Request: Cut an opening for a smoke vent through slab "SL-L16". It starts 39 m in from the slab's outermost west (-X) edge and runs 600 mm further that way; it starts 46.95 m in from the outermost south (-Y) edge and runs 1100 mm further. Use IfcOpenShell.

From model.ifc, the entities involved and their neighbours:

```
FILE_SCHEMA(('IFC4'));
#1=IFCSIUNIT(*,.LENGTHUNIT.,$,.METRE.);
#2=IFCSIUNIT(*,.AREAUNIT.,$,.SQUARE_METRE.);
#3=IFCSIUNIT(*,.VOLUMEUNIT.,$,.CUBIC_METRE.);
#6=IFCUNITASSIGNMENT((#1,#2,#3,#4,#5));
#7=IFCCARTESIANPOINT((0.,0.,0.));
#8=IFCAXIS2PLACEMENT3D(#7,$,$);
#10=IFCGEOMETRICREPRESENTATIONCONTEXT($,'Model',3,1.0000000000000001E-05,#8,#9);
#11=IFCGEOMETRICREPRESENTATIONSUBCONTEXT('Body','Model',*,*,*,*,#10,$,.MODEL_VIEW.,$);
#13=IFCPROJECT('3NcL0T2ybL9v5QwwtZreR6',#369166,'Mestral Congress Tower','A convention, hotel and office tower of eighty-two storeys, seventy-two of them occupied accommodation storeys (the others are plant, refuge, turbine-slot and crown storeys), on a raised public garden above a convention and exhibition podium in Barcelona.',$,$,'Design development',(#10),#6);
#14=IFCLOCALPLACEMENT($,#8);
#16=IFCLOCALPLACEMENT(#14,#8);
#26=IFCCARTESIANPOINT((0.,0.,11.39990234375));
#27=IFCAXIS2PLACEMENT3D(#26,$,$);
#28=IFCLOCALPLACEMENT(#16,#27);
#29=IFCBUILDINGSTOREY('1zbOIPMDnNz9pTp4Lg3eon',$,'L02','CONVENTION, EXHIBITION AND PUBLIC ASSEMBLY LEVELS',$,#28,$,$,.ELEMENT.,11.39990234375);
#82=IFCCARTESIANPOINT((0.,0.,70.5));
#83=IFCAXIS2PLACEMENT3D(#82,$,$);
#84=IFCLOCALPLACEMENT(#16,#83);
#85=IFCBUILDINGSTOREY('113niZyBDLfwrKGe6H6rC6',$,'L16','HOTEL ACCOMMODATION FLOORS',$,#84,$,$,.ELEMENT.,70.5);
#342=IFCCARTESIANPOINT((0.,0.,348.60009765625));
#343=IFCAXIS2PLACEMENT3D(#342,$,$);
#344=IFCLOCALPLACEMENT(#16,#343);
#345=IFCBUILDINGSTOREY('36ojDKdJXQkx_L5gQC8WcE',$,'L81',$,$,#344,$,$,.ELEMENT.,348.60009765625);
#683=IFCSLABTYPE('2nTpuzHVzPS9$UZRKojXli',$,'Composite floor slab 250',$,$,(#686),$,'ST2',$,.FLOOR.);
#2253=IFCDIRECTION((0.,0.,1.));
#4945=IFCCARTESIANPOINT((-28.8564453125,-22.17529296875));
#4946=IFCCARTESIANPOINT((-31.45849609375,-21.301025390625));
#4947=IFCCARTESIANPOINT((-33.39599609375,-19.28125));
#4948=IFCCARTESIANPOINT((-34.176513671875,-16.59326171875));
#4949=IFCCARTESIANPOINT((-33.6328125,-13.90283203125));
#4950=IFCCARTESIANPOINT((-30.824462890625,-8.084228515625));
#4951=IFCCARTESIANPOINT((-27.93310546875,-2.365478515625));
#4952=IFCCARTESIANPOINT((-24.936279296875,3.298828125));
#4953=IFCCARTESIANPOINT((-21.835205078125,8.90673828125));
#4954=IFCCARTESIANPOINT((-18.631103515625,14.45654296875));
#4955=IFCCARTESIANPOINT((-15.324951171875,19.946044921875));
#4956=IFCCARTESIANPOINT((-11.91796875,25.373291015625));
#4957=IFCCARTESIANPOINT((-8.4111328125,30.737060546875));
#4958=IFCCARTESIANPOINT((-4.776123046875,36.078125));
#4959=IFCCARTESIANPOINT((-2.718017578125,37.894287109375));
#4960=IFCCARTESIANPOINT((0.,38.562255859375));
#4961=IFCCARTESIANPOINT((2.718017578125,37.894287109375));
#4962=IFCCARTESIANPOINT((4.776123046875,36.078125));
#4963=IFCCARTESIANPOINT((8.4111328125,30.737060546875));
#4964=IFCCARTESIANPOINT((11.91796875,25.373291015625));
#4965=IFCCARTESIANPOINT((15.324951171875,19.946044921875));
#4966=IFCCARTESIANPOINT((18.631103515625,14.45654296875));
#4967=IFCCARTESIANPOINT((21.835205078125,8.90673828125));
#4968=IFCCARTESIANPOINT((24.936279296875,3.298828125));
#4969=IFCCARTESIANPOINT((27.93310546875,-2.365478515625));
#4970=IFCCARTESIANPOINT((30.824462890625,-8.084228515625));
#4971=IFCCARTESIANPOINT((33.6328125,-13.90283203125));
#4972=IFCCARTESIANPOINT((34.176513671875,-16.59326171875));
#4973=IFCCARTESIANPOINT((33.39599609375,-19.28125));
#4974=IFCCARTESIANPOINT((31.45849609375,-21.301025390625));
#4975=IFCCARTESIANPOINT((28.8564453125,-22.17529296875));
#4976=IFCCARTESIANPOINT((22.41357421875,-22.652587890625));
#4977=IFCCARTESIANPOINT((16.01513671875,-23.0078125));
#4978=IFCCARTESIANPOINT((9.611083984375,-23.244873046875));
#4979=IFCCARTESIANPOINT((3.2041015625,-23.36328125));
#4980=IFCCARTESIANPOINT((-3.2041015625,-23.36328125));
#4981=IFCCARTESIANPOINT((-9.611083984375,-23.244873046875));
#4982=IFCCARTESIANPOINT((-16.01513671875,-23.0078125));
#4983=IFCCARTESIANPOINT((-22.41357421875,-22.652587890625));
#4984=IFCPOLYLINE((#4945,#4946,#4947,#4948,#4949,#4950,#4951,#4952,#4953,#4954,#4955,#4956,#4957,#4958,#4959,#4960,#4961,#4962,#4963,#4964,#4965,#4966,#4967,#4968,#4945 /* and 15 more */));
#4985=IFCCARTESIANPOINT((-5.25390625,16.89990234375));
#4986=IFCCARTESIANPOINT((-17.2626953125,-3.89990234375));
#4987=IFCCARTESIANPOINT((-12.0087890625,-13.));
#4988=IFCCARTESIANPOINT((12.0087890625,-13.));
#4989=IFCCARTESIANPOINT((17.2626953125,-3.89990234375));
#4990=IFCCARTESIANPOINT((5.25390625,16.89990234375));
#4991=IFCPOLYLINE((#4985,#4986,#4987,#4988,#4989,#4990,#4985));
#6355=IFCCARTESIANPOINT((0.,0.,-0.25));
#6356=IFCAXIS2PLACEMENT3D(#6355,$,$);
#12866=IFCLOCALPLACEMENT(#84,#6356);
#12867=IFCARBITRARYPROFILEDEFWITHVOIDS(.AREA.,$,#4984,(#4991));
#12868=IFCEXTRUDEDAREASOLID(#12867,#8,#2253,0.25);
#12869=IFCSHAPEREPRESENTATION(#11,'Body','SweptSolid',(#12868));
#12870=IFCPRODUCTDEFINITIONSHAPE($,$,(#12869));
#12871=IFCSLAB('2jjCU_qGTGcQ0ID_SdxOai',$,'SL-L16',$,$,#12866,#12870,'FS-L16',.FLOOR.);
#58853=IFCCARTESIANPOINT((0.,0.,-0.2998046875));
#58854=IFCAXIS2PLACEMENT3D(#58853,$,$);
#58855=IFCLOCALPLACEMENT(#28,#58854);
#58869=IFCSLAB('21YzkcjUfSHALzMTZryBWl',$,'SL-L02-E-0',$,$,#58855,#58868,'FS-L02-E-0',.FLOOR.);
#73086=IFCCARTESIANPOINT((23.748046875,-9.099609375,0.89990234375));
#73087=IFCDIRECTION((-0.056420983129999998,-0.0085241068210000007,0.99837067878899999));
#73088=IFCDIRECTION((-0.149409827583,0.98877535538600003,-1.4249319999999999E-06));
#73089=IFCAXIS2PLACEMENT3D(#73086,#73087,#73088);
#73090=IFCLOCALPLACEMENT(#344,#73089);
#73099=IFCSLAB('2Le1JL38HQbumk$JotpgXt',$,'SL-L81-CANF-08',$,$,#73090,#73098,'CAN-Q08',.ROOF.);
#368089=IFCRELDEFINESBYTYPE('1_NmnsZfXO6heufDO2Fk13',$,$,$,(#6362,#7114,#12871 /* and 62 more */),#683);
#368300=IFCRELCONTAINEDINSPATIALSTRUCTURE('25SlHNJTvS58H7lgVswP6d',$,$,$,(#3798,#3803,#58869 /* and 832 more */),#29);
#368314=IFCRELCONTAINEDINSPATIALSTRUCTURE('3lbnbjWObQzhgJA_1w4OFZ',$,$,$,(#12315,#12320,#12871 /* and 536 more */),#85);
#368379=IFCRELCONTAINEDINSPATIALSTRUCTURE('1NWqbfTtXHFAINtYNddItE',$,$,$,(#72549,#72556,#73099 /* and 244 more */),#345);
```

```python
import numpy as np
import ifcopenshell
import ifcopenshell.api.feature
import ifcopenshell.api.geometry
import ifcopenshell.api.root
import ifcopenshell.geom
import ifcopenshell.util.placement
import ifcopenshell.util.representation
import ifcopenshell.util.shape
import ifcopenshell.util.unit

model = ifcopenshell.open("model.ifc")
unit_scale = ifcopenshell.util.unit.calculate_unit_scale(model)
settings = ifcopenshell.geom.settings()


def volume(element):
    """Net volume in cubic metres, openings subtracted."""
    shape = ifcopenshell.geom.create_shape(settings, element)
    return ifcopenshell.util.shape.get_volume(shape.geometry)


slab = model.by_guid("2jjCU_qGTGcQ0ID_SdxOai")
before = volume(slab)

# Extent in the slab's own axes, in metres. The edges named are its -X and -Y sides.
slab_shape = ifcopenshell.geom.create_shape(settings, slab)
vertices = ifcopenshell.util.shape.get_vertices(slab_shape.geometry)
x_min, y_min, bottom = vertices.min(axis=0)
top = vertices[:, 2].max()

opening = ifcopenshell.api.root.create_entity(model, ifc_class="IfcOpeningElement", name="Smoke vent opening", predefined_type="OPENING")
context = ifcopenshell.util.representation.get_context(model, "Model", "Body", "MODEL_VIEW")
width, depth = 0.6, 1.1
outline = [(0.0, 0.0), (width, 0.0), (width, depth), (0.0, depth), (0.0, 0.0)]
# Overshoot both faces by 50 mm so the cut is clean.
shape = ifcopenshell.api.geometry.add_slab_representation(
    model, context=context, depth=top - bottom + 0.1, polyline=outline
)
ifcopenshell.api.geometry.assign_representation(model, product=opening, representation=shape)

matrix = ifcopenshell.util.placement.get_local_placement(slab.ObjectPlacement)
matrix[:, 3] = matrix @ np.append(np.array([x_min + 39, y_min + 46.95, bottom - 0.05]) / unit_scale, 1.0)
ifcopenshell.api.geometry.edit_object_placement(model, product=opening, matrix=matrix, is_si=False)
ifcopenshell.api.feature.add_feature(model, feature=opening, element=slab)

after = volume(slab)

print(f"slab volume {before:.3f} -> {after:.3f} m3")

model.write("model-out.ifc")
```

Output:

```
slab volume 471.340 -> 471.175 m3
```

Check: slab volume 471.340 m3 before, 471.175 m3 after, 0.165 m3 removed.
